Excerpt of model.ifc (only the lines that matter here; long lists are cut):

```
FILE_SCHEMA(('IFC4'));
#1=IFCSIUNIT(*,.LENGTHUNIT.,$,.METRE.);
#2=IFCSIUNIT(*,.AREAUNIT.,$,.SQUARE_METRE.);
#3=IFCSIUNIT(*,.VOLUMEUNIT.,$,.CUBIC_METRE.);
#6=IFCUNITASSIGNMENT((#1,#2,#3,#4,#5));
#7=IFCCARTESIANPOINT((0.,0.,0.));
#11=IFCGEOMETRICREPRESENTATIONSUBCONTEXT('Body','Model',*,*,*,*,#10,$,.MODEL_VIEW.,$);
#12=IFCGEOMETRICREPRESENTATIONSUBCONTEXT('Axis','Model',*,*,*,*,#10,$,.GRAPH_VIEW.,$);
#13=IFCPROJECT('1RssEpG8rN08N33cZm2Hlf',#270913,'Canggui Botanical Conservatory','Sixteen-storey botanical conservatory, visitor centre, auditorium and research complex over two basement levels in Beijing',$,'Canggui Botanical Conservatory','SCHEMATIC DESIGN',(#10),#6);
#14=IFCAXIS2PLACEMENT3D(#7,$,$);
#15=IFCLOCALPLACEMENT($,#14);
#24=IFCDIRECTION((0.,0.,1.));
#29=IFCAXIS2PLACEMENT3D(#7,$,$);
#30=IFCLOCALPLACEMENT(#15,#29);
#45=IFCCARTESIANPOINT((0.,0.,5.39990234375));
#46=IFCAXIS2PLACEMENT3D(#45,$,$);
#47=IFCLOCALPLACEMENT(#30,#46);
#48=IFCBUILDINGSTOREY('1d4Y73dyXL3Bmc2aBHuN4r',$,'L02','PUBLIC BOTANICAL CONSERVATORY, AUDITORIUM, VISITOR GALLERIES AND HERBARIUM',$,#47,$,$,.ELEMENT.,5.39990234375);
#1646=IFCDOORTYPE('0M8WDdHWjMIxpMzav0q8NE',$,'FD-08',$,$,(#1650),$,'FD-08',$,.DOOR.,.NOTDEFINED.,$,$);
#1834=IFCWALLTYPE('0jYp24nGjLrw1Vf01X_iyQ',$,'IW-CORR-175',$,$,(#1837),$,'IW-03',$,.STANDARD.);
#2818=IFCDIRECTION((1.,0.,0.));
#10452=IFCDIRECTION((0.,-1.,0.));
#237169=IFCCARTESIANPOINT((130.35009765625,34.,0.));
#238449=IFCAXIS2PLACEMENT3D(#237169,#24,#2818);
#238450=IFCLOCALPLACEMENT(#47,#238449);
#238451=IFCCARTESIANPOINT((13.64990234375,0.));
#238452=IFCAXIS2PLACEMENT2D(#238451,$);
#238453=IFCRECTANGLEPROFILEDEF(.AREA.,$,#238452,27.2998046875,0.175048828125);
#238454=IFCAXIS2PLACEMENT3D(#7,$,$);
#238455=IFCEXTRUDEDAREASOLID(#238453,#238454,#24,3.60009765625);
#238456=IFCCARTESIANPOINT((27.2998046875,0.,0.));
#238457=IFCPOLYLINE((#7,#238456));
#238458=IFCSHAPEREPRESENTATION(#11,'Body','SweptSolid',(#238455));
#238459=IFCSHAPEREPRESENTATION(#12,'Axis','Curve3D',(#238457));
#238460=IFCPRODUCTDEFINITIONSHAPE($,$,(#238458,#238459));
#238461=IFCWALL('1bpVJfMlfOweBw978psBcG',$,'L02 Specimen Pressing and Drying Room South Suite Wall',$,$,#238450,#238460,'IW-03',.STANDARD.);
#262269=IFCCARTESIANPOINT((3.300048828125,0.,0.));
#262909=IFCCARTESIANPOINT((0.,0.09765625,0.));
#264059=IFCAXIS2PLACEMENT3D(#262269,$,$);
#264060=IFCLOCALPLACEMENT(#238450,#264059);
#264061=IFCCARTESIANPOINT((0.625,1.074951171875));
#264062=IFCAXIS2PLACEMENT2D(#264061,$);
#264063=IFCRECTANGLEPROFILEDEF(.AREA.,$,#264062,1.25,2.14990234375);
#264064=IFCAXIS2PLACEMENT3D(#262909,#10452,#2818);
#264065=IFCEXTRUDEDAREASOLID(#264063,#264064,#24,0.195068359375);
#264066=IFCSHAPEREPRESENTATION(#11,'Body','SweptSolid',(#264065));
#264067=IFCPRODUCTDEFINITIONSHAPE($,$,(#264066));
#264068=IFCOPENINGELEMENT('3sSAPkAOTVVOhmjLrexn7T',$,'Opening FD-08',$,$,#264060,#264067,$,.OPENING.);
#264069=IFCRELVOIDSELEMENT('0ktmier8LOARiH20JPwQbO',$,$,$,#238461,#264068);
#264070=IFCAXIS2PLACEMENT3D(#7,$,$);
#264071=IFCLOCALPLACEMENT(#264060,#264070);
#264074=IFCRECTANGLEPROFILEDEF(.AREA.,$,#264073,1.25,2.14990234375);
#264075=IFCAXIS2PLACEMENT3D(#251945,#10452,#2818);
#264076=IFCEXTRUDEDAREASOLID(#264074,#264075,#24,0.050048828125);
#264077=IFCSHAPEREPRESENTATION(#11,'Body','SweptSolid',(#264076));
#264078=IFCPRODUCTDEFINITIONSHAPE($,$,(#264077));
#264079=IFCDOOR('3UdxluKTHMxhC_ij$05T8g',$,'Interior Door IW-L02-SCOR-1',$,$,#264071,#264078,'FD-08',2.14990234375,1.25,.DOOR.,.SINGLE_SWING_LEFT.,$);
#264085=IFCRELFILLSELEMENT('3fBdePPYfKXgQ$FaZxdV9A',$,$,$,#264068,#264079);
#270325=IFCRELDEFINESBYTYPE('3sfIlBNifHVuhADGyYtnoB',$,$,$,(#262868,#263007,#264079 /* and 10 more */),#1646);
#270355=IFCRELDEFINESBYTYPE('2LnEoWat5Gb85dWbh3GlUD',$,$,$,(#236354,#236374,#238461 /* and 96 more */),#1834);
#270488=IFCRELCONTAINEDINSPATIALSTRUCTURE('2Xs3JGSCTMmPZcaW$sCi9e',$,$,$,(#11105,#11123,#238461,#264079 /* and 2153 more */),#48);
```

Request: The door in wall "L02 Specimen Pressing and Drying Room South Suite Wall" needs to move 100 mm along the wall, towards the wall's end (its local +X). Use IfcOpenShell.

```python
import ifcopenshell
import ifcopenshell.api.geometry
import ifcopenshell.util.placement
import ifcopenshell.util.unit

model = ifcopenshell.open("model.ifc")
unit_scale = ifcopenshell.util.unit.calculate_unit_scale(model)

door = model.by_guid("3UdxluKTHMxhC_ij$05T8g")
opening = door.FillsVoids[0].RelatingOpeningElement
wall = opening.VoidsElements[0].RelatingBuildingElement

wall_matrix = ifcopenshell.util.placement.get_local_placement(wall.ObjectPlacement)
shift = wall_matrix[:3, 0] * 0.1 / unit_scale
before = ifcopenshell.util.placement.get_local_placement(door.ObjectPlacement)[:3, 3].copy()

# The door is placed relative to its opening, so it follows when the opening moves.
matrix = ifcopenshell.util.placement.get_local_placement(opening.ObjectPlacement)
matrix[:3, 3] += shift
ifcopenshell.api.geometry.edit_object_placement(
    model, product=opening, matrix=matrix, is_si=False, should_transform_children=True
)

after = ifcopenshell.util.placement.get_local_placement(door.ObjectPlacement)[:3, 3]
print("door moved by", (after - before).round(3) + 0.0)

model.write("model_rev.ifc")
```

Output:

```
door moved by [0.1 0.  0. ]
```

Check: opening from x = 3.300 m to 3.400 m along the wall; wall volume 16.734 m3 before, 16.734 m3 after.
